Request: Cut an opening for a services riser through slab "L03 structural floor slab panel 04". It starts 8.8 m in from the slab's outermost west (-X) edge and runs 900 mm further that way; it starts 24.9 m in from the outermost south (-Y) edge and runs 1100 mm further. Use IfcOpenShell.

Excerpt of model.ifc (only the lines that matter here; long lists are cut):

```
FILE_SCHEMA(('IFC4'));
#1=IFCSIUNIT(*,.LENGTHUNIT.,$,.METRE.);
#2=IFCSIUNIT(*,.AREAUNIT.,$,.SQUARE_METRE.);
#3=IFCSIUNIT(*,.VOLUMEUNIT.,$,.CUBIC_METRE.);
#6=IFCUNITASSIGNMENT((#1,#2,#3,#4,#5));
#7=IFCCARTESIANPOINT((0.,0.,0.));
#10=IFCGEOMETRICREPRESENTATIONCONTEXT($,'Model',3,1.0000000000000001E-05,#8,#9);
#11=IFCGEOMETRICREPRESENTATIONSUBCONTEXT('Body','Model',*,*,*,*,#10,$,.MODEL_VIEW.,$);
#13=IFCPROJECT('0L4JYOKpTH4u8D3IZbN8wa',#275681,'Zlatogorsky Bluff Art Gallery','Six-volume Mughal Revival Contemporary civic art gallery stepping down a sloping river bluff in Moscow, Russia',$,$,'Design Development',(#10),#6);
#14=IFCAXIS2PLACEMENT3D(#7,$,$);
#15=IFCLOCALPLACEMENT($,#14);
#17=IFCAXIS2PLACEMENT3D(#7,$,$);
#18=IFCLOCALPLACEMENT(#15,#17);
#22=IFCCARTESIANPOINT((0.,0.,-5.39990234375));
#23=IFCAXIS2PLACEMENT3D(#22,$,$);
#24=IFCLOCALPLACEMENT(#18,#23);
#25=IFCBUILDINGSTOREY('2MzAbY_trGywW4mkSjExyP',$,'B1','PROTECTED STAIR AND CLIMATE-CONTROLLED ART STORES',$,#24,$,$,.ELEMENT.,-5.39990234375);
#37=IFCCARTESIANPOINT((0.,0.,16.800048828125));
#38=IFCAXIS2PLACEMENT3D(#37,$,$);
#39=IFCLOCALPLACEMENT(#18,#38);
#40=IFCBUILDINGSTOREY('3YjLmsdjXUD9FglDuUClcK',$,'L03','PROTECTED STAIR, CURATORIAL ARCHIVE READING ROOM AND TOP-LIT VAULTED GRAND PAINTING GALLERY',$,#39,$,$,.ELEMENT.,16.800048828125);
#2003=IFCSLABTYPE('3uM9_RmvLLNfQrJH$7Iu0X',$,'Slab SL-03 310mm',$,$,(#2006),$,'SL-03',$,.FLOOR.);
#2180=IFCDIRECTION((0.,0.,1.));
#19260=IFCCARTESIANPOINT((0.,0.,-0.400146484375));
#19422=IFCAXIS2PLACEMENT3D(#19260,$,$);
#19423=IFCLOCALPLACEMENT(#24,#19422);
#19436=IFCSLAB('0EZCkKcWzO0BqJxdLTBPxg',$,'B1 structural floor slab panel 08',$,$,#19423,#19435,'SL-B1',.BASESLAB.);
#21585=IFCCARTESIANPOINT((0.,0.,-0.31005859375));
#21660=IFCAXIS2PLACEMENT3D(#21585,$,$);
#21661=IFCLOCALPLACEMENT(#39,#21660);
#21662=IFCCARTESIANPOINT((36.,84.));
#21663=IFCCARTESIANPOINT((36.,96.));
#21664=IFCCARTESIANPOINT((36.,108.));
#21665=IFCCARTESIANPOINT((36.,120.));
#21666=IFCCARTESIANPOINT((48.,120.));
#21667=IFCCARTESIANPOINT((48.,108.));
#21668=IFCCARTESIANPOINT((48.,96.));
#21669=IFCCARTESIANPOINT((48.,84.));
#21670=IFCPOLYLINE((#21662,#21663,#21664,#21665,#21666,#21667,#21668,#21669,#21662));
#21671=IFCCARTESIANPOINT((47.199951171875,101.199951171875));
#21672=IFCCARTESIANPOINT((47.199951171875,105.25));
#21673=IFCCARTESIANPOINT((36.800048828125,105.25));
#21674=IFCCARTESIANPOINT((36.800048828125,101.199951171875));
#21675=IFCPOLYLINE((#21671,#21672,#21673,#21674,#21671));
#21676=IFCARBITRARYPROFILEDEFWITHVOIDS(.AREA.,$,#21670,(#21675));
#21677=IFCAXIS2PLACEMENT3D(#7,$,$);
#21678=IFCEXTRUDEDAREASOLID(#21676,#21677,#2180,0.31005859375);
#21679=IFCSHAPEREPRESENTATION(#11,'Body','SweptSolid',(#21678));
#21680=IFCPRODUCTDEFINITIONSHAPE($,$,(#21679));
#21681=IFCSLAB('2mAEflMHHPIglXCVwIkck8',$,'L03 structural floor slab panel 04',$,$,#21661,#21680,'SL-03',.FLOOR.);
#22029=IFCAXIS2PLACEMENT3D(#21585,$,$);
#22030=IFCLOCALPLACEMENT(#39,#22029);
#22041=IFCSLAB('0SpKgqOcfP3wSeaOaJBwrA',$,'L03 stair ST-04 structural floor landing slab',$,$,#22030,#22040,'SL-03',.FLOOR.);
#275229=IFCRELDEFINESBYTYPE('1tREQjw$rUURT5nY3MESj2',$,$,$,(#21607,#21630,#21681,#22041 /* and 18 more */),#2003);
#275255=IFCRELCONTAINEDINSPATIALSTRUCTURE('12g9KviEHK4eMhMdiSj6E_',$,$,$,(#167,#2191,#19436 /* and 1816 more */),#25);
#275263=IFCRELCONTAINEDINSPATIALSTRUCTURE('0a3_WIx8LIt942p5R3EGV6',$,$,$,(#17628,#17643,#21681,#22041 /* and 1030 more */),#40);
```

```python
import numpy as np
import ifcopenshell
import ifcopenshell.api.feature
import ifcopenshell.api.geometry
import ifcopenshell.api.root
import ifcopenshell.geom
import ifcopenshell.util.placement
import ifcopenshell.util.representation
import ifcopenshell.util.shape
import ifcopenshell.util.unit

model = ifcopenshell.open("model.ifc")
unit_scale = ifcopenshell.util.unit.calculate_unit_scale(model)
settings = ifcopenshell.geom.settings()


def volume(element):
    """Net volume in cubic metres, openings subtracted."""
    shape = ifcopenshell.geom.create_shape(settings, element)
    return ifcopenshell.util.shape.get_volume(shape.geometry)


slab = model.by_guid("2mAEflMHHPIglXCVwIkck8")
before = volume(slab)

# Extent in the slab's own axes, in metres. The edges named are its -X and -Y sides.
slab_shape = ifcopenshell.geom.create_shape(settings, slab)
vertices = ifcopenshell.util.shape.get_vertices(slab_shape.geometry)
x_min, y_min, bottom = vertices.min(axis=0)
top = vertices[:, 2].max()

opening = ifcopenshell.api.root.create_entity(model, ifc_class="IfcOpeningElement", name="Services riser opening", predefined_type="OPENING")
context = ifcopenshell.util.representation.get_context(model, "Model", "Body", "MODEL_VIEW")
width, depth = 0.9, 1.1
outline = [(0.0, 0.0), (width, 0.0), (width, depth), (0.0, depth), (0.0, 0.0)]
# Overshoot both faces by 50 mm so the cut is clean.
shape = ifcopenshell.api.geometry.add_slab_representation(
    model, context=context, depth=top - bottom + 0.1, polyline=outline
)
ifcopenshell.api.geometry.assign_representation(model, product=opening, representation=shape)

matrix = ifcopenshell.util.placement.get_local_placement(slab.ObjectPlacement)
matrix[:, 3] = matrix @ np.append(np.array([x_min + 8.8, y_min + 24.9, bottom - 0.05]) / unit_scale, 1.0)
ifcopenshell.api.geometry.edit_object_placement(model, product=opening, matrix=matrix, is_si=False)
ifcopenshell.api.feature.add_feature(model, feature=opening, element=slab)

after = volume(slab)

print(f"slab volume {before:.3f} -> {after:.3f} m3")

model.write("model_rev.ifc")
```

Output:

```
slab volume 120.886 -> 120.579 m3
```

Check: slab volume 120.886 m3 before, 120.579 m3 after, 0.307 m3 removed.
